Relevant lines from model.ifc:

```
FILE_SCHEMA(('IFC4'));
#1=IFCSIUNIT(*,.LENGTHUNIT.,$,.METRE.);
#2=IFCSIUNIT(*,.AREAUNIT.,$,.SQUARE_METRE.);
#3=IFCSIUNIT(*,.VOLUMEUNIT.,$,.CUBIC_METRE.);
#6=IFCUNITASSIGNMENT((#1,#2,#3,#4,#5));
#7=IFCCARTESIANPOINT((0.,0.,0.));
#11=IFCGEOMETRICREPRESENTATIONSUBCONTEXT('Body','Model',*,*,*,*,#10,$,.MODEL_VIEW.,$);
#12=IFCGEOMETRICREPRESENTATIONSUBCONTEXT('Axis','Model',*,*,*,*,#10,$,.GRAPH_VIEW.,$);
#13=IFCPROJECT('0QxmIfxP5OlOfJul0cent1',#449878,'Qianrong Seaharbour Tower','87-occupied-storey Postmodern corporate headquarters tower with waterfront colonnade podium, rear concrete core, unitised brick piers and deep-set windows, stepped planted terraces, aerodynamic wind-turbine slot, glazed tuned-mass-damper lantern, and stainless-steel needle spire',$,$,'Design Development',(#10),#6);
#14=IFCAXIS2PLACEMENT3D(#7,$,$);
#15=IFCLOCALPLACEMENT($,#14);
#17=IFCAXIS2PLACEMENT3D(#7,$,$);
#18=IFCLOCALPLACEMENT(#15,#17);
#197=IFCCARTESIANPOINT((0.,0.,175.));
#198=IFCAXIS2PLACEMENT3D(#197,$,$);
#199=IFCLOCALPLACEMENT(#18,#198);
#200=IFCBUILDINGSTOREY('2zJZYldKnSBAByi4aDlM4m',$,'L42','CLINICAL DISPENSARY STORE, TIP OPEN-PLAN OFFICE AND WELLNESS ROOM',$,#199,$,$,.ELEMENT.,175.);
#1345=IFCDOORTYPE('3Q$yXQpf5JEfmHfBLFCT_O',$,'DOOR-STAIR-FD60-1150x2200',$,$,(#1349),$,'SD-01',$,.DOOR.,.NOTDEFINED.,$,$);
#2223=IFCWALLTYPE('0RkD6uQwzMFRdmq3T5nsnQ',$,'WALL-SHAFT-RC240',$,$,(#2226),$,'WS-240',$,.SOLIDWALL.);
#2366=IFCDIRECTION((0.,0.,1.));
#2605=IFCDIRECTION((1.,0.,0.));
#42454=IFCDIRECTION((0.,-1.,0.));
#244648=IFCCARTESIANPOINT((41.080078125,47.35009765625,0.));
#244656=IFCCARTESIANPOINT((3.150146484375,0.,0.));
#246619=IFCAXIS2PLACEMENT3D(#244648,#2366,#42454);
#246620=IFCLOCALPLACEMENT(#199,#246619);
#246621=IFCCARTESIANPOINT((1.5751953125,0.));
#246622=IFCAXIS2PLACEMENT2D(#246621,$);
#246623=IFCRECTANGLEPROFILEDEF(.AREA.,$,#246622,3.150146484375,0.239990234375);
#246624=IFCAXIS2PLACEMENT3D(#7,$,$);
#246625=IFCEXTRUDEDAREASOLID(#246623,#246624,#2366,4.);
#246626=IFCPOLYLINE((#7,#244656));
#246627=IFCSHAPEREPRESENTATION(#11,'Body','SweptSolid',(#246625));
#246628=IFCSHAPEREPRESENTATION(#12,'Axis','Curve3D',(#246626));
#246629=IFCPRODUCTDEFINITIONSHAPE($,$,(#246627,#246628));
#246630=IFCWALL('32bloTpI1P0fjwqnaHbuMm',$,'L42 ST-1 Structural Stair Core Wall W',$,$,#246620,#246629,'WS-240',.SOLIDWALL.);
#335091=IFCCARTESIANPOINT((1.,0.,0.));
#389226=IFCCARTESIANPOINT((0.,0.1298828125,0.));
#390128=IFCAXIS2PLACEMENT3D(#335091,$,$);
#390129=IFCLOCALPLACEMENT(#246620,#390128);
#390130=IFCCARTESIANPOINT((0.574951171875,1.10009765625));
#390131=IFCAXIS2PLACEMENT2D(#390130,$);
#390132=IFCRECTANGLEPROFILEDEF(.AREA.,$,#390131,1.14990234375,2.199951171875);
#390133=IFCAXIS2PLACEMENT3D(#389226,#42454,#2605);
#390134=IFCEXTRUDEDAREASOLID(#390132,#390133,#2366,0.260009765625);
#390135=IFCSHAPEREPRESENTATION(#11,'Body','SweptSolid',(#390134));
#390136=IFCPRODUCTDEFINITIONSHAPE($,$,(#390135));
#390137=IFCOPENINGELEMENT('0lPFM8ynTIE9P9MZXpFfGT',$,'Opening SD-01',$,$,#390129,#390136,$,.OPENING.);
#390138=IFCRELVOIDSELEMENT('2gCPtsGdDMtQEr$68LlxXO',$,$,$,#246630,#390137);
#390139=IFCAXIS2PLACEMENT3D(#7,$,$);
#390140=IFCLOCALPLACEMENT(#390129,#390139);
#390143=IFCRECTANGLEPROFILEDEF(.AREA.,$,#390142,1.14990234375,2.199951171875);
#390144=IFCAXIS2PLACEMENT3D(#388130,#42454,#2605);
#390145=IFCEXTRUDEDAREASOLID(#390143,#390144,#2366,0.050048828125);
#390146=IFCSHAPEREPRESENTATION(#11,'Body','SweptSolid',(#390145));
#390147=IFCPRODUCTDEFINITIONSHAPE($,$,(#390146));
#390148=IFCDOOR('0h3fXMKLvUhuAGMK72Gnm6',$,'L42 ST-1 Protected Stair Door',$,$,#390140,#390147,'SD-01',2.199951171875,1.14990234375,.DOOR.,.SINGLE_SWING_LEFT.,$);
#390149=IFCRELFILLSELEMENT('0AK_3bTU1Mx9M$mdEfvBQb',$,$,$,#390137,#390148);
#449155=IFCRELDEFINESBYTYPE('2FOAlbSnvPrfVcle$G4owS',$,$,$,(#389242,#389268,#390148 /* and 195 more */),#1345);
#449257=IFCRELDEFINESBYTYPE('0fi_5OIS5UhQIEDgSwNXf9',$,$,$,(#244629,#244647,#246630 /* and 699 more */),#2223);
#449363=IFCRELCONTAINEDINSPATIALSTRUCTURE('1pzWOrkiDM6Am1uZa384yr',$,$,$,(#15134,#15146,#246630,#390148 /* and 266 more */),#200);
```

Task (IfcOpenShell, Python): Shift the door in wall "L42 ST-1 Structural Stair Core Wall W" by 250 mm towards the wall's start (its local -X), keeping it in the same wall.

```python
import ifcopenshell
import ifcopenshell.api.geometry
import ifcopenshell.util.placement
import ifcopenshell.util.unit

model = ifcopenshell.open("model.ifc")
unit_scale = ifcopenshell.util.unit.calculate_unit_scale(model)

door = model.by_id(390148)
opening = door.FillsVoids[0].RelatingOpeningElement
wall = opening.VoidsElements[0].RelatingBuildingElement

wall_matrix = ifcopenshell.util.placement.get_local_placement(wall.ObjectPlacement)
shift = wall_matrix[:3, 0] * -0.25 / unit_scale
before = ifcopenshell.util.placement.get_local_placement(door.ObjectPlacement)[:3, 3].copy()

# The door is placed relative to its opening, so it follows when the opening moves.
matrix = ifcopenshell.util.placement.get_local_placement(opening.ObjectPlacement)
matrix[:3, 3] += shift
ifcopenshell.api.geometry.edit_object_placement(
    model, product=opening, matrix=matrix, is_si=False, should_transform_children=True
)

after = ifcopenshell.util.placement.get_local_placement(door.ObjectPlacement)[:3, 3]
print("door moved by", (after - before).round(3) + 0.0)

model.write("model_rev.ifc")
```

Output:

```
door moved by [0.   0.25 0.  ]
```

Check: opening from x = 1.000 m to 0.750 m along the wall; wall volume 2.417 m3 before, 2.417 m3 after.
